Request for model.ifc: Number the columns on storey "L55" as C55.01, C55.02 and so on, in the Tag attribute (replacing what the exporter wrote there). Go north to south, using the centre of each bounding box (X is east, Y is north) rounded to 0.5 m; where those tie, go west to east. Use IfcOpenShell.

First a look at what the model holds.

```python
import ifcopenshell
import ifcopenshell.util.element
import ifcopenshell.util.placement

model = ifcopenshell.open("model.ifc")
print(model.schema)
storey = next(s for s in model.by_type("IfcBuildingStorey") if s.Name == "L55")
columns = [e for e in ifcopenshell.util.element.get_decomposition(storey) if e.is_a("IfcColumn")]
for e in sorted(columns, key=lambda e: e.id()):
    origin = ifcopenshell.util.placement.get_local_placement(e.ObjectPlacement)[:3, 3]
    print(e.id(), e.Tag, e.Name, origin.round(2) + 0.0, sep=" | ")
```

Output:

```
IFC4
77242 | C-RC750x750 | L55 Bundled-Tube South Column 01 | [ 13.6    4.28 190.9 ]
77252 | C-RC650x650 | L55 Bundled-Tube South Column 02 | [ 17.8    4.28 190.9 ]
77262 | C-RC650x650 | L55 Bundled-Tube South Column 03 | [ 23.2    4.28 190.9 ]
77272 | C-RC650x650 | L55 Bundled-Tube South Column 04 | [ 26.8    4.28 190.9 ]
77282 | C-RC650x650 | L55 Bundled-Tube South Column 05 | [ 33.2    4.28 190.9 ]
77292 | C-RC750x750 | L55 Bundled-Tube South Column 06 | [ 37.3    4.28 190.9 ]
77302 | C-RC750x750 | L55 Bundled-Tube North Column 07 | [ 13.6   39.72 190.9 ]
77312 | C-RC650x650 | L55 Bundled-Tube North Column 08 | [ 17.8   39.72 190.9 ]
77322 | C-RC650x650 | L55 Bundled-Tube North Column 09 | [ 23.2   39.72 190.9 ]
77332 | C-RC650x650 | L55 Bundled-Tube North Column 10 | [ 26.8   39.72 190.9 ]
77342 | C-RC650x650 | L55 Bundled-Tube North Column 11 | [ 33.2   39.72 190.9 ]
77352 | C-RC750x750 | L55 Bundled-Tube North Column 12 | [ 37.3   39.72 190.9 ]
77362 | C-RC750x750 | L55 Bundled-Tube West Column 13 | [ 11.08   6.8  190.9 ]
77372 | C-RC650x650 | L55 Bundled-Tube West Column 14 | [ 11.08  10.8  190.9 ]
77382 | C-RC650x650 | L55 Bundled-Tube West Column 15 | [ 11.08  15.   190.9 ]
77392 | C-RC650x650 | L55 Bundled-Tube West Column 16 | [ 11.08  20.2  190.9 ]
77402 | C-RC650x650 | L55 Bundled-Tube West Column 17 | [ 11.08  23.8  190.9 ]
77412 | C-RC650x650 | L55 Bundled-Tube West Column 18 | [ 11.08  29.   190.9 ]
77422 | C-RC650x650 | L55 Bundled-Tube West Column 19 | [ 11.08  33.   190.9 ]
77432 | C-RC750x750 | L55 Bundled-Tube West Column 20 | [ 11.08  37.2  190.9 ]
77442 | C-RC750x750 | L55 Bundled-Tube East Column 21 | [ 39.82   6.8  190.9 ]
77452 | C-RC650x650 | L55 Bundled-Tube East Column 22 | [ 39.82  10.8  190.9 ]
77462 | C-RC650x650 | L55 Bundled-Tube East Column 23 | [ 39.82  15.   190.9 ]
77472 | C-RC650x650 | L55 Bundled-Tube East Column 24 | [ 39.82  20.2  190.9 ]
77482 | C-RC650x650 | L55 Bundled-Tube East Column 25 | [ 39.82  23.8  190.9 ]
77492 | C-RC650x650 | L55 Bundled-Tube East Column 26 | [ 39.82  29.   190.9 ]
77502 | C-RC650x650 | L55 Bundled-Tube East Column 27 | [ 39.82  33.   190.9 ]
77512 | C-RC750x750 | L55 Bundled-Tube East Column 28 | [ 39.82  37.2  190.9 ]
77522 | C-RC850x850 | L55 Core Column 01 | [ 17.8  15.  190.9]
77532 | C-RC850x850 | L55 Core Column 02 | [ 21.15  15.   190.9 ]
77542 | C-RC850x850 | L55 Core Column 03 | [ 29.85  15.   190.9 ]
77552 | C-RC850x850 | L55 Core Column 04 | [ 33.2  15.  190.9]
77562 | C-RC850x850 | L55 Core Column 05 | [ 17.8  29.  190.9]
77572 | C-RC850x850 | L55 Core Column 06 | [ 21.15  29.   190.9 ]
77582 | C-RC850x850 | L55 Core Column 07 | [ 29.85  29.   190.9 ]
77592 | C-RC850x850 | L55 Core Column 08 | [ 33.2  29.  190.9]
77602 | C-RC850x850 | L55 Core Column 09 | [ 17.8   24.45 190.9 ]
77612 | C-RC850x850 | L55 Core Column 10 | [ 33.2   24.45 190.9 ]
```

```python
import ifcopenshell
import ifcopenshell.geom
import ifcopenshell.util.element
import ifcopenshell.util.shape

model = ifcopenshell.open("model.ifc")
settings = ifcopenshell.geom.settings()
settings.set("use-world-coords", True)


def centre(element):
    shape = ifcopenshell.geom.create_shape(settings, element)
    return ifcopenshell.util.shape.get_bbox_centroid(shape.geometry)


storey = next(s for s in model.by_type("IfcBuildingStorey") if s.Name == "L55")
columns = [e for e in ifcopenshell.util.element.get_decomposition(storey) if e.is_a("IfcColumn")]

# Insertion points can sit at a corner or the storey origin, so sort by the geometry (in metres).
centres = {e: centre(e) for e in columns}
columns.sort(key=lambda e: (-round(centres[e][1] / 0.5), centres[e][0]))

for i, e in enumerate(columns, start=1):
    number = f"C55.{i:02d}"
    e.Tag = number
    print(e.id(), number)

model.write("model_edited.ifc")
```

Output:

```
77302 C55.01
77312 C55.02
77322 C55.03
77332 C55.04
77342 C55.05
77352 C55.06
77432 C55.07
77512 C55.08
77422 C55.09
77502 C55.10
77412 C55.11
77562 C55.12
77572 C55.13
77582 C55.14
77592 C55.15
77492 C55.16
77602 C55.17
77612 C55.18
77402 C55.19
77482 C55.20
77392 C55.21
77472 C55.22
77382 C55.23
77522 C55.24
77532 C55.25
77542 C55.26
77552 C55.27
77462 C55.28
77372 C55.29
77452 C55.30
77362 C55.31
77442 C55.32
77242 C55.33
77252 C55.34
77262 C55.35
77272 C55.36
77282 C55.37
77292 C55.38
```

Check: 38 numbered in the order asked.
